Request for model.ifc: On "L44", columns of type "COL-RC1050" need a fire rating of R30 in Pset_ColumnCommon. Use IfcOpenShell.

First a look at what the model holds.

```python
import ifcopenshell
import ifcopenshell.util.element

model = ifcopenshell.open("model.ifc")
print(model.schema)
storey = next(s for s in model.by_type("IfcBuildingStorey") if s.Name == "L44")
columns = [e for e in ifcopenshell.util.element.get_decomposition(storey) if e.is_a("IfcColumn")]
seen = {}
for e in columns:
    element_type = ifcopenshell.util.element.get_type(e)
    key = (element_type.Name if element_type != e and element_type else None, ifcopenshell.util.element.get_pset(e, "Pset_ColumnCommon", "FireRating"))
    seen[key] = seen.get(key, 0) + 1
for (name, value), count in sorted(seen.items(), key=str):
    print(count, "x", name, "|", value)
```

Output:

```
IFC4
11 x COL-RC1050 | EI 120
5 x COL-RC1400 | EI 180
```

```python
import ifcopenshell
import ifcopenshell.api.pset
import ifcopenshell.util.element

model = ifcopenshell.open("model.ifc")

storey = next(s for s in model.by_type("IfcBuildingStorey") if s.Name == "L44")
columns = [e for e in ifcopenshell.util.element.get_decomposition(storey) if e.is_a("IfcColumn")]

count = 0
for e in columns:
    element_type = ifcopenshell.util.element.get_type(e)
    if element_type in (None, e) or element_type.Name != "COL-RC1050":
        continue
    found = ifcopenshell.util.element.get_pset(e, "Pset_ColumnCommon", should_inherit=False)
    if found:
        pset = model.by_id(found["id"])
        if len(ifcopenshell.util.element.get_elements_by_pset(pset)) > 1:
            pset = ifcopenshell.api.pset.unshare_pset(model, products=[e], pset=pset)[0]
    else:
        pset = ifcopenshell.api.pset.add_pset(model, product=e, name="Pset_ColumnCommon")
    ifcopenshell.api.pset.edit_pset(model, pset=pset, properties={"FireRating": "R30"})
    count += 1

print(count, "columns updated")

model.write("model_v2.ifc")
```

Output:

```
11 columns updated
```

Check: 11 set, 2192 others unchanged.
